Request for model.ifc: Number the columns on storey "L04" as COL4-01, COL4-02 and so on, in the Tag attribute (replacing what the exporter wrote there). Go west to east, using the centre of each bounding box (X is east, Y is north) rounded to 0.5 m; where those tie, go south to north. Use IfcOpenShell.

First a look at what the model holds.

```python
import ifcopenshell
import ifcopenshell.util.element
import ifcopenshell.util.placement

model = ifcopenshell.open("model.ifc")
print(model.schema)
storey = next(s for s in model.by_type("IfcBuildingStorey") if s.Name == "L04")
columns = [e for e in ifcopenshell.util.element.get_decomposition(storey) if e.is_a("IfcColumn")]
for e in sorted(columns, key=lambda e: e.id()):
    origin = ifcopenshell.util.placement.get_local_placement(e.ObjectPlacement)[:3, 3]
    print(e.id(), e.Tag, e.Name, origin.round(2) + 0.0, sep=" | ")
```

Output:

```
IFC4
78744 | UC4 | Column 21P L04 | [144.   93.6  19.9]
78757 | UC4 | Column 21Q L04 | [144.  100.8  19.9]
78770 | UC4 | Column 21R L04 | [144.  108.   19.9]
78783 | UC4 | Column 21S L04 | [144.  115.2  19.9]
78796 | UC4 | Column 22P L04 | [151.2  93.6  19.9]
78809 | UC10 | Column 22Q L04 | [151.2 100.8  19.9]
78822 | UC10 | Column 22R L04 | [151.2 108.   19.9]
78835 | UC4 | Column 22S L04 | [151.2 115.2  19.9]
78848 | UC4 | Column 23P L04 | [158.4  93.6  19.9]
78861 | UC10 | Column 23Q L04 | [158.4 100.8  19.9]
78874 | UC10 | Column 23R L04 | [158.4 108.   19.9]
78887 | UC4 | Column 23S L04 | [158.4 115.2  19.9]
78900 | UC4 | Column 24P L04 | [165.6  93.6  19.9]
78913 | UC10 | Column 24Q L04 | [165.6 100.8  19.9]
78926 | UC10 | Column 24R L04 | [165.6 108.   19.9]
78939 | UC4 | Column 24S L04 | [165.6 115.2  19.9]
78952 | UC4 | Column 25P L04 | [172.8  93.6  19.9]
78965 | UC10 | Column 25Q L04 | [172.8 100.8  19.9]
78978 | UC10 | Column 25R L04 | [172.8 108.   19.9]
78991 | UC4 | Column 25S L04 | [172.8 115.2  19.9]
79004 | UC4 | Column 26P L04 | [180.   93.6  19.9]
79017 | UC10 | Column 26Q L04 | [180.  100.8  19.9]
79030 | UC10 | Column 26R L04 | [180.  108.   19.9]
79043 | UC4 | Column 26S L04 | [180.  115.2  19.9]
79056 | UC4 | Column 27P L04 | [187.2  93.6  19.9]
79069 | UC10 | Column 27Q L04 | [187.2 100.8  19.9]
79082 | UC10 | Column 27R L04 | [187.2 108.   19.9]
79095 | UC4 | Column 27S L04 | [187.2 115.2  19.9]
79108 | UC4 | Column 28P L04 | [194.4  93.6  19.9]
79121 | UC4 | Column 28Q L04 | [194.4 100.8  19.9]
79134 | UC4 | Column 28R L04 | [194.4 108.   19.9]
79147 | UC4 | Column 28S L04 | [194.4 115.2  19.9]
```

```python
import ifcopenshell
import ifcopenshell.geom
import ifcopenshell.util.element
import ifcopenshell.util.shape

model = ifcopenshell.open("model.ifc")
settings = ifcopenshell.geom.settings()
settings.set("use-world-coords", True)


def centre(element):
    shape = ifcopenshell.geom.create_shape(settings, element)
    return ifcopenshell.util.shape.get_bbox_centroid(shape.geometry)


storey = next(s for s in model.by_type("IfcBuildingStorey") if s.Name == "L04")
columns = [e for e in ifcopenshell.util.element.get_decomposition(storey) if e.is_a("IfcColumn")]

# Insertion points can sit at a corner or the storey origin, so sort by the geometry (in metres).
centres = {e: centre(e) for e in columns}
columns.sort(key=lambda e: (round(centres[e][0] / 0.5), centres[e][1]))

for i, e in enumerate(columns, start=1):
    number = f"COL4-{i:02d}"
    e.Tag = number
    print(e.id(), number)

model.write("model-out.ifc")
```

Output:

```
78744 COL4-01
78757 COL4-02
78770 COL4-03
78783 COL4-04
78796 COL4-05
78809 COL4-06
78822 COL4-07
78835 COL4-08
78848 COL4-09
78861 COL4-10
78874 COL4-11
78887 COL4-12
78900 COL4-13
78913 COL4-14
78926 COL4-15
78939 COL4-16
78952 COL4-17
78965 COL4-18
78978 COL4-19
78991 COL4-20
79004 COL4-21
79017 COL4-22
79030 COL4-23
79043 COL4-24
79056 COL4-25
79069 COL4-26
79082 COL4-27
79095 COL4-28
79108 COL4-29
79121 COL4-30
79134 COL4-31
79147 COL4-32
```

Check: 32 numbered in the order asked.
